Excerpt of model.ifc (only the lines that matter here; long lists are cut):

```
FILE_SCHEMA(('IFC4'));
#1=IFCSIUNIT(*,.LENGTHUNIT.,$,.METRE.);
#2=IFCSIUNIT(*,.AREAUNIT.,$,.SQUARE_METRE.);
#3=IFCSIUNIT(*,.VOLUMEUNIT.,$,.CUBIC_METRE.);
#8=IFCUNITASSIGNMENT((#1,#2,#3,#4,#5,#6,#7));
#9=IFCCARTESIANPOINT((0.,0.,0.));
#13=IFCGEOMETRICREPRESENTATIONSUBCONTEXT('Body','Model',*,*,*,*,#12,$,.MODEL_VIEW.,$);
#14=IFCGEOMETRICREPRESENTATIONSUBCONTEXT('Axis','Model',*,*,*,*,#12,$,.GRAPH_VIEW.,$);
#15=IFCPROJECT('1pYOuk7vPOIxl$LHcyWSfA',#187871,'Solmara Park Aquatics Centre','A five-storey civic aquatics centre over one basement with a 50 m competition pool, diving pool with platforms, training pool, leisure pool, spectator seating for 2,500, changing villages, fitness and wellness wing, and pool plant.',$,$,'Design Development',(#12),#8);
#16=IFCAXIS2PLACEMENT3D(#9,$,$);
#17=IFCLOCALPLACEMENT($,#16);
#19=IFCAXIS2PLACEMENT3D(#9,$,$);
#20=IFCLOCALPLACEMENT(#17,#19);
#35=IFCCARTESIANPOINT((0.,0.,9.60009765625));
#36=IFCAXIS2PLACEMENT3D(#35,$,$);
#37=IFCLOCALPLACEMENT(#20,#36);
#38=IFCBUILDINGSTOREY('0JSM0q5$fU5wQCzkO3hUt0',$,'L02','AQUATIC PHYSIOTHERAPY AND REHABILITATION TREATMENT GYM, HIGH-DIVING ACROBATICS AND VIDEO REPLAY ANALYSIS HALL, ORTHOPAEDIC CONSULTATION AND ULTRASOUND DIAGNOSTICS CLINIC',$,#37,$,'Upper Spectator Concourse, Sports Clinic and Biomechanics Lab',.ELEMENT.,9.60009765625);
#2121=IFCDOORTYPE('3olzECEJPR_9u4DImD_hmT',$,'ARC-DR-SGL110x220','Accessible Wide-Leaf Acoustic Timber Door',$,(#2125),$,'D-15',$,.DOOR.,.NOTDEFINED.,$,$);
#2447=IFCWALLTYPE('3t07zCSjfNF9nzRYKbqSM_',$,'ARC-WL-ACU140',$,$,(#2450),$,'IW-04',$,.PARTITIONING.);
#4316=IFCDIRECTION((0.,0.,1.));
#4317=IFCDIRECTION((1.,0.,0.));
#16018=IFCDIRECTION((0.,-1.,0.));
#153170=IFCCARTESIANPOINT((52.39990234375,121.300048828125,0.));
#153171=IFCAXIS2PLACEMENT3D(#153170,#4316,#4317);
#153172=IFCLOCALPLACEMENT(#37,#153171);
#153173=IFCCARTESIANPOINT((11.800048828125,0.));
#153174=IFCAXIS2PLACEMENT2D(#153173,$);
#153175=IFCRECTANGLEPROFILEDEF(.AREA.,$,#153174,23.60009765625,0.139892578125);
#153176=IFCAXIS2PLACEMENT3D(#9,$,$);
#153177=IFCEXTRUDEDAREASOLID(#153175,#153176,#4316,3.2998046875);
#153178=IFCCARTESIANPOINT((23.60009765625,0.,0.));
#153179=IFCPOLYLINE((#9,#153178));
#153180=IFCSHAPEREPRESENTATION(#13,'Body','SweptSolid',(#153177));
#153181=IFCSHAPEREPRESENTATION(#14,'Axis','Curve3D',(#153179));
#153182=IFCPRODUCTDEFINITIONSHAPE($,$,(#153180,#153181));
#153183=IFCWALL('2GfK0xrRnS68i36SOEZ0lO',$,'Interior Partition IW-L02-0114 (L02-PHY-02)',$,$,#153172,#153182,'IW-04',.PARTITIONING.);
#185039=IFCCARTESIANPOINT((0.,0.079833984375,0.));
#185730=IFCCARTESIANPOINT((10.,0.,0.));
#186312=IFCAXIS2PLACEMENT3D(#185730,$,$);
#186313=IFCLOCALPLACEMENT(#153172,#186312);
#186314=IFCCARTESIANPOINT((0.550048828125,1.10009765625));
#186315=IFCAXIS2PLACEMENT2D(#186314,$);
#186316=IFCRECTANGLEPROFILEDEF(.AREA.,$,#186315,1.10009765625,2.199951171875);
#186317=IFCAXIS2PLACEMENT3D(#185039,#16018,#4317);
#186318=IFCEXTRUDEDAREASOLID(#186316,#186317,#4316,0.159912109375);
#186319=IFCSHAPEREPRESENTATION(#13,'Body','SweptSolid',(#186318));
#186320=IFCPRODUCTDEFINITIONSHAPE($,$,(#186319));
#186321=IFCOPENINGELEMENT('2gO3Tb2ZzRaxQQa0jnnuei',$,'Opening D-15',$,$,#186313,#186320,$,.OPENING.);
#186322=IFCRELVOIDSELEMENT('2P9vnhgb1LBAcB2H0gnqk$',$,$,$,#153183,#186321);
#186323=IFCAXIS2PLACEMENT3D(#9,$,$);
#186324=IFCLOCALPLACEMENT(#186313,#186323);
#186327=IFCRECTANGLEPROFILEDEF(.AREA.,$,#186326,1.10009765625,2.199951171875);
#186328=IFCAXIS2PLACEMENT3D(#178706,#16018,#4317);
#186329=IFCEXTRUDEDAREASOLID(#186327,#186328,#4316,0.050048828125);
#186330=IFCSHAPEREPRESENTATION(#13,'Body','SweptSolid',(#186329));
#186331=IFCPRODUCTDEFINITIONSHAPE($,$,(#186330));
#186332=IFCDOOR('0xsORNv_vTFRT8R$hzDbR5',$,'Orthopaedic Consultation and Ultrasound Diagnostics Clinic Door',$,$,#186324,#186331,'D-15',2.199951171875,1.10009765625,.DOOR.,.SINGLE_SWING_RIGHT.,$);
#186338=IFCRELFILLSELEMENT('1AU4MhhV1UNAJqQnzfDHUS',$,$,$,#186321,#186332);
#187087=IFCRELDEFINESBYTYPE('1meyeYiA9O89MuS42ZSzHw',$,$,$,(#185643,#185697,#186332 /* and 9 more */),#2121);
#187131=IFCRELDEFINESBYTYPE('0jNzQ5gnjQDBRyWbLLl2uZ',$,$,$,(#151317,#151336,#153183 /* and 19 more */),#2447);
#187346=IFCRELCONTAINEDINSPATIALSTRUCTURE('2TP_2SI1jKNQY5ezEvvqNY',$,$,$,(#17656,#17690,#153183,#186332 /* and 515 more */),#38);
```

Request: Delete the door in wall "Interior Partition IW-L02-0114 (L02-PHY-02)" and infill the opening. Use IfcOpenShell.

```python
import ifcopenshell
import ifcopenshell.api.feature
import ifcopenshell.api.root
import ifcopenshell.geom
import ifcopenshell.util.shape

model = ifcopenshell.open("model.ifc")
settings = ifcopenshell.geom.settings()


def volume(element):
    """Net volume in cubic metres, openings subtracted."""
    shape = ifcopenshell.geom.create_shape(settings, element)
    return ifcopenshell.util.shape.get_volume(shape.geometry)


door = model.by_guid("0xsORNv_vTFRT8R$hzDbR5")
opening = door.FillsVoids[0].RelatingOpeningElement
wall = opening.VoidsElements[0].RelatingBuildingElement
before = volume(wall)

ifcopenshell.api.root.remove_product(model, product=door)
ifcopenshell.api.feature.remove_feature(model, feature=opening)

after = volume(wall)

print(f"wall volume {before:.3f} -> {after:.3f} m3")

model.write("model_rev.ifc")
```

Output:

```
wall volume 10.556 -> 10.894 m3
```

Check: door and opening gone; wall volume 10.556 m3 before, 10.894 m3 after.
